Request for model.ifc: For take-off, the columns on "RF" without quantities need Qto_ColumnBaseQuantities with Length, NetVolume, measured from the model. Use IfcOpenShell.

First a look at what the model holds.

```python
import ifcopenshell
import ifcopenshell.util.element
import ifcopenshell.util.unit

model = ifcopenshell.open("model.ifc")
print(model.schema)
for unit_type in ("LENGTHUNIT", "AREAUNIT", "VOLUMEUNIT"):
    print(unit_type, ifcopenshell.util.unit.calculate_unit_scale(model, unit_type))
storey = next(s for s in model.by_type("IfcBuildingStorey") if s.Name == "RF")
columns = [e for e in ifcopenshell.util.element.get_decomposition(storey) if e.is_a("IfcColumn")]
for e in sorted(columns, key=lambda e: e.id()):
    print(e.id(), e.is_a(), e.Name, list(ifcopenshell.util.element.get_psets(e, qtos_only=True)), sep=" | ")
```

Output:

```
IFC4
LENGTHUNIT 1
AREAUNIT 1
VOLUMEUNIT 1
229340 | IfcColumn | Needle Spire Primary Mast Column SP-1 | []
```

```python
import ifcopenshell
import ifcopenshell.api.pset
import ifcopenshell.geom
import ifcopenshell.util.element
import ifcopenshell.util.shape
import ifcopenshell.util.unit

model = ifcopenshell.open("model.ifc")
unit_scale = ifcopenshell.util.unit.calculate_unit_scale(model)
volume_scale = ifcopenshell.util.unit.calculate_unit_scale(model, "VOLUMEUNIT")
settings = ifcopenshell.geom.settings()

storey = next(s for s in model.by_type("IfcBuildingStorey") if s.Name == "RF")
columns = [e for e in ifcopenshell.util.element.get_decomposition(storey) if e.is_a("IfcColumn")]

for e in sorted(columns, key=lambda e: e.id()):
    if ifcopenshell.util.element.get_psets(e, qtos_only=True, should_inherit=False):
        continue
    # Geometry comes back in metres, in the element's own axes.
    shape = ifcopenshell.geom.create_shape(settings, e)
    values = {
        "Length": ifcopenshell.util.shape.get_z(shape.geometry) / unit_scale,
        "NetVolume": ifcopenshell.util.shape.get_volume(shape.geometry) / volume_scale,
    }
    qto = ifcopenshell.api.pset.add_qto(model, product=e, name="Qto_ColumnBaseQuantities")
    ifcopenshell.api.pset.edit_qto(model, qto=qto, properties=values)
    print(e.id(), {k: round(v, 3) for k, v in values.items()})

model.write("model_rev.ifc")
```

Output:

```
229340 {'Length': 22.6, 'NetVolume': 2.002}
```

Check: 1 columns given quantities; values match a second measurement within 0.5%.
